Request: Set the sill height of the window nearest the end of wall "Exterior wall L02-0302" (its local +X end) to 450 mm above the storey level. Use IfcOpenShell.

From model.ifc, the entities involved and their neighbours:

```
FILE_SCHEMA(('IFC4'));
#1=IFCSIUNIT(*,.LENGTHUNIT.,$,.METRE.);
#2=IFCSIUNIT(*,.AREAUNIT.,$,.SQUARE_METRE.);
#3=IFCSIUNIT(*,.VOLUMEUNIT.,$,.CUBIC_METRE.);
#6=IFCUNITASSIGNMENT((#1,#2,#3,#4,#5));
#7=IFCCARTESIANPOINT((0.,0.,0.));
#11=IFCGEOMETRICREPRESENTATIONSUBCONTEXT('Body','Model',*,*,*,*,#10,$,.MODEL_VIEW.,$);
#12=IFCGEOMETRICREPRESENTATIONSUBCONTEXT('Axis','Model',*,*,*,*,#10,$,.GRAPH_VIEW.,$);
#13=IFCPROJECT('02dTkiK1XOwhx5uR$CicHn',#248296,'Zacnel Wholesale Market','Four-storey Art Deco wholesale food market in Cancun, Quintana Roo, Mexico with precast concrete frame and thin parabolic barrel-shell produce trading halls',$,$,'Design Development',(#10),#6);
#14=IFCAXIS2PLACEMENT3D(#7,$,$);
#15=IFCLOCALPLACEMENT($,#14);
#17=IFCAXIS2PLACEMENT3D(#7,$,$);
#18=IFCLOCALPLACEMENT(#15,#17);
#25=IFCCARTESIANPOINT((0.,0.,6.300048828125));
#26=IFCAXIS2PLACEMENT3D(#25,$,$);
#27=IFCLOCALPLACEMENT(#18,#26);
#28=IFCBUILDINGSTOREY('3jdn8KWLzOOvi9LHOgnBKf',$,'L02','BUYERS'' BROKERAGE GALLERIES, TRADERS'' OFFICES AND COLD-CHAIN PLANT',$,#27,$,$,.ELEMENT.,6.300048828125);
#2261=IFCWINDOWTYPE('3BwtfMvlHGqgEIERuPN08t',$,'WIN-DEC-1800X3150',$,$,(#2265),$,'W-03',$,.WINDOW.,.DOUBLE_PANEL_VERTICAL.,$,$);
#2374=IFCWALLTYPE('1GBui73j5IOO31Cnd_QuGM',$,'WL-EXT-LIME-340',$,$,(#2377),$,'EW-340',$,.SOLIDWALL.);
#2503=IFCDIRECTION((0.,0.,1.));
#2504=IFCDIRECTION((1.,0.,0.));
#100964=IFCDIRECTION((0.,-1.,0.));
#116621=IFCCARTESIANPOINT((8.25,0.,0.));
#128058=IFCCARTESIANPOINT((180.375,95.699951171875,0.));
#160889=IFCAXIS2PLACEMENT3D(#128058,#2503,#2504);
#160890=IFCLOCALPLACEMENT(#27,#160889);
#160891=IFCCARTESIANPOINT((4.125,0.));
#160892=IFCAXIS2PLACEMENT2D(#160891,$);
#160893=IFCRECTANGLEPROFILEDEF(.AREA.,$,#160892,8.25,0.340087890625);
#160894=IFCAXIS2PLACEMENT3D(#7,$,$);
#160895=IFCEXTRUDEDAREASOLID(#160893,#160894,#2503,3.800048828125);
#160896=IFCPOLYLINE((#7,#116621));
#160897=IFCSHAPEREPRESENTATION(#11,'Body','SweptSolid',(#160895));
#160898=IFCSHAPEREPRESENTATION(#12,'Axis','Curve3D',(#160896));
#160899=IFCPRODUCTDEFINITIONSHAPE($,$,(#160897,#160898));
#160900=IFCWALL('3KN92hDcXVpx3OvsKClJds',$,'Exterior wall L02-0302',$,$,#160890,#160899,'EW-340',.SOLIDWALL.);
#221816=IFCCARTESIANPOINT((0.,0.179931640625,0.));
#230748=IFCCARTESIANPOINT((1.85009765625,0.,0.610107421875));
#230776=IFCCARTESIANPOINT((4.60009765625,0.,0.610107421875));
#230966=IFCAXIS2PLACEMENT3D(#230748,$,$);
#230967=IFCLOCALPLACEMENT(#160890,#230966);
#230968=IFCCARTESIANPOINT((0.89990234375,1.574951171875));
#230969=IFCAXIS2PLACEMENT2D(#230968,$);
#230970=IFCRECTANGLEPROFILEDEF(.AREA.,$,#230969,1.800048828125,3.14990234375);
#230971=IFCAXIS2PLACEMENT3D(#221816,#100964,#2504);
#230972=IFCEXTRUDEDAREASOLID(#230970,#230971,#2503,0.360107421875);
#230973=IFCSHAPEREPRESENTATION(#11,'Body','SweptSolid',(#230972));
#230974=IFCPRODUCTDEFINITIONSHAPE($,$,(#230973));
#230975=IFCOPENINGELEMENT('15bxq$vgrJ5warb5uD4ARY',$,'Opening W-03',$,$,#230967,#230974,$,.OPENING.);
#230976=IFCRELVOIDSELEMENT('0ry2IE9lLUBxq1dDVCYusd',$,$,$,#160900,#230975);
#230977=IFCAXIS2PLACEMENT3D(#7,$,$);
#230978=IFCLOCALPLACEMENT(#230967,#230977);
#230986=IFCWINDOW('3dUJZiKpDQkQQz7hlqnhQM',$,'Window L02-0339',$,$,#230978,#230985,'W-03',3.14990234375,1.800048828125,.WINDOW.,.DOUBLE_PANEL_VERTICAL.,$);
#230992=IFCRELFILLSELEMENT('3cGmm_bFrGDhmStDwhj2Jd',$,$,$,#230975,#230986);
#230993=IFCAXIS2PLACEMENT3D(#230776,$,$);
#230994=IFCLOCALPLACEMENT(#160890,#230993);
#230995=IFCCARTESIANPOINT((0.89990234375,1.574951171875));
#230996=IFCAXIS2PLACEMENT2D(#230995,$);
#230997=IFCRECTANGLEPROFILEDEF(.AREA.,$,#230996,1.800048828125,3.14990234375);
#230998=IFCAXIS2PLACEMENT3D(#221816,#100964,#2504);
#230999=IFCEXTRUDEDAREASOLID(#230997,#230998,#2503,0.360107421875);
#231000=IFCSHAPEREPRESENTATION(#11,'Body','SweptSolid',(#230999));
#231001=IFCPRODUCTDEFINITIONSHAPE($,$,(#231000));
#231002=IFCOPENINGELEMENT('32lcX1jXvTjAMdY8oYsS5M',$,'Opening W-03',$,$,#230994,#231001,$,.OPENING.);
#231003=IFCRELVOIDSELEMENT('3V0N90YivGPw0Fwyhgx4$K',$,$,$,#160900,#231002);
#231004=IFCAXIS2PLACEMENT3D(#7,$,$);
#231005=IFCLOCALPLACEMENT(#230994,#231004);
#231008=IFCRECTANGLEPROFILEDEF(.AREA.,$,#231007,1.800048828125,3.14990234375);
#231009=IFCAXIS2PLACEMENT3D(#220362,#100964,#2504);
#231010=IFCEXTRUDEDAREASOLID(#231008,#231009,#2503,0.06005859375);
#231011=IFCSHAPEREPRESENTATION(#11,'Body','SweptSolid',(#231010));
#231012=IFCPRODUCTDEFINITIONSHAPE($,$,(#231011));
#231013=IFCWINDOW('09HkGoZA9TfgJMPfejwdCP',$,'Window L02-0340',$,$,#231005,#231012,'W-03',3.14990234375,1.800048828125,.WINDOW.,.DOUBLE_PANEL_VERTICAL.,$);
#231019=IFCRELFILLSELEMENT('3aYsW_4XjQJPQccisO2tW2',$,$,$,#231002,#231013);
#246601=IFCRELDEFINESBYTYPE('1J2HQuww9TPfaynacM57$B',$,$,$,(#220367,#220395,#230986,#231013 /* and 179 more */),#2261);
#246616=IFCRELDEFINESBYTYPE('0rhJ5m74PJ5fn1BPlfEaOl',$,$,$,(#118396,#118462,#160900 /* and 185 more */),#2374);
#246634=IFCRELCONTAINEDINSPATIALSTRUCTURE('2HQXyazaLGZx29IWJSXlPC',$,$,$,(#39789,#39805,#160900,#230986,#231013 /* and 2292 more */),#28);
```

```python
import numpy as np
import ifcopenshell
import ifcopenshell.api.geometry
import ifcopenshell.geom
import ifcopenshell.util.element
import ifcopenshell.util.placement
import ifcopenshell.util.shape
import ifcopenshell.util.unit

model = ifcopenshell.open("model.ifc")
unit_scale = ifcopenshell.util.unit.calculate_unit_scale(model)

window = model.by_guid("09HkGoZA9TfgJMPfejwdCP")
opening = window.FillsVoids[0].RelatingOpeningElement
storey = ifcopenshell.util.element.get_container(window, ifc_class="IfcBuildingStorey")
level = ifcopenshell.util.placement.get_local_placement(storey.ObjectPlacement)[2, 3]

# The opening's origin need not be at the sill, so measure its lowest point.
shape = ifcopenshell.geom.create_shape(ifcopenshell.geom.settings(), opening)
bottom = ifcopenshell.util.shape.get_shape_bottom_elevation(shape, shape.geometry) / unit_scale
dz = level + 0.45 - bottom

shift = np.array([0.0, 0.0, dz])
# The window is placed relative to its opening, so it follows when the opening moves.
matrix = ifcopenshell.util.placement.get_local_placement(opening.ObjectPlacement)
matrix[:3, 3] += shift
ifcopenshell.api.geometry.edit_object_placement(
    model, product=opening, matrix=matrix, is_si=False, should_transform_children=True
)

print(f"moved by {dz * unit_scale:+.3f} m")

model.write("model_edited.ifc")
```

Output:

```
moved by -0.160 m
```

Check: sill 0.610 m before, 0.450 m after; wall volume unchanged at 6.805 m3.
